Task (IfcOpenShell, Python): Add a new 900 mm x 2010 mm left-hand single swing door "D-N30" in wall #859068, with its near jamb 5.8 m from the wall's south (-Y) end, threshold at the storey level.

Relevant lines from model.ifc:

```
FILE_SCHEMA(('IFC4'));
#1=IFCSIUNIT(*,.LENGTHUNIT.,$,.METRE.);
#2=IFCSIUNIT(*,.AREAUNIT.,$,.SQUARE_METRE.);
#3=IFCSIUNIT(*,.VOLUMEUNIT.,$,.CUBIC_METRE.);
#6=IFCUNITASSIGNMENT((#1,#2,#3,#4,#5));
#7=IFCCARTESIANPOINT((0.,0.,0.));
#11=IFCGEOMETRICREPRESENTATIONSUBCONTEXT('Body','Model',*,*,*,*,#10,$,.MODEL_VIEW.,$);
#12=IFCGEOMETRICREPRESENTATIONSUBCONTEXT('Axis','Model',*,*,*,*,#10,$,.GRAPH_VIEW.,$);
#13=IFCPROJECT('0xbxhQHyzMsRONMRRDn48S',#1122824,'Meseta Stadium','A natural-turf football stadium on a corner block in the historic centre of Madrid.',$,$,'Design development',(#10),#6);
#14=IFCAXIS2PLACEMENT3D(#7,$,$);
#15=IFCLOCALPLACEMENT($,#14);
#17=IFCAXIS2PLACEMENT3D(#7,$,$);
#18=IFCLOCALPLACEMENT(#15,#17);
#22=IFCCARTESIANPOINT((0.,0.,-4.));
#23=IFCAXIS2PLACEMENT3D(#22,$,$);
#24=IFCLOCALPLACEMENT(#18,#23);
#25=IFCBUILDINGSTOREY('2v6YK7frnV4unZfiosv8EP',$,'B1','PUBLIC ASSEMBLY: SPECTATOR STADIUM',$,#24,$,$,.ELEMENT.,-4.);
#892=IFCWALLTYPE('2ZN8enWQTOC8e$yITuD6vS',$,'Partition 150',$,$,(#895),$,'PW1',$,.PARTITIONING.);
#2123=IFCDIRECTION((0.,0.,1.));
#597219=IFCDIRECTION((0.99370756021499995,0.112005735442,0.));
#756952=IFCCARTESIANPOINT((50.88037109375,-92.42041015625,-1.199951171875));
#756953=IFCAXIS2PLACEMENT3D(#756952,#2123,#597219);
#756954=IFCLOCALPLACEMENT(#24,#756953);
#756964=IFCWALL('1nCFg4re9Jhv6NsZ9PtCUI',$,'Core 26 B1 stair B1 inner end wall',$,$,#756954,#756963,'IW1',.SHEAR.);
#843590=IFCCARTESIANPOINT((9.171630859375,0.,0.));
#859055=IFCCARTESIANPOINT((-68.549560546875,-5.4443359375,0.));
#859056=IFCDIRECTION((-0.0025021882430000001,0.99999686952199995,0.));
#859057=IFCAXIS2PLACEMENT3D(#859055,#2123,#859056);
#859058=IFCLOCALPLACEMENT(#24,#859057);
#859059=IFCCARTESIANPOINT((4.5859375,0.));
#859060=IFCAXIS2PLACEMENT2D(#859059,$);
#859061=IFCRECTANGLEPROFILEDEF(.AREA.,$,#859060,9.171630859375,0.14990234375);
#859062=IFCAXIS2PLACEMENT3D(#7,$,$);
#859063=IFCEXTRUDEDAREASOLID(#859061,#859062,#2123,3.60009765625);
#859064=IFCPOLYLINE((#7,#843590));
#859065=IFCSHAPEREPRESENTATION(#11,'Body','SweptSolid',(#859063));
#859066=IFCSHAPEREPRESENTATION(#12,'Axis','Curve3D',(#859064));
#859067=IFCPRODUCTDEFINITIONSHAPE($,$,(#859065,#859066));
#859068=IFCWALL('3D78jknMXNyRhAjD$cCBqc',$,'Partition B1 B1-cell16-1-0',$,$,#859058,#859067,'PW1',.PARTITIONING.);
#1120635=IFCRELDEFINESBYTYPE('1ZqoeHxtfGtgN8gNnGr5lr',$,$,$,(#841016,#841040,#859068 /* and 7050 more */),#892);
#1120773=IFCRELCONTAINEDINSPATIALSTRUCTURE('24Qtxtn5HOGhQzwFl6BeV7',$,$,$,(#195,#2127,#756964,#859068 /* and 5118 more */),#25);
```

```python
import numpy as np
import ifcopenshell
import ifcopenshell.api.feature
import ifcopenshell.api.geometry
import ifcopenshell.api.root
import ifcopenshell.api.spatial
import ifcopenshell.geom
import ifcopenshell.util.element
import ifcopenshell.util.placement
import ifcopenshell.util.representation
import ifcopenshell.util.shape
import ifcopenshell.util.unit

model = ifcopenshell.open("model.ifc")
unit_scale = ifcopenshell.util.unit.calculate_unit_scale(model)
settings = ifcopenshell.geom.settings()


def volume(element):
    """Net volume in cubic metres, openings subtracted."""
    shape = ifcopenshell.geom.create_shape(settings, element)
    return ifcopenshell.util.shape.get_volume(shape.geometry)


wall = model.by_id(859068)
storey = ifcopenshell.util.element.get_container(wall, ifc_class="IfcBuildingStorey")
context = ifcopenshell.util.representation.get_context(model, "Model", "Body", "MODEL_VIEW")
before = volume(wall)

width, height, from_end, sill = 0.9, 2.01, 5.8, 0.0  # metres

# The wall runs along its own X axis, and the end named is its -X end.
wall_shape = ifcopenshell.geom.create_shape(settings, wall)
x, y, z = ifcopenshell.util.shape.get_vertices(wall_shape.geometry).T
start = x.min() + from_end
face, thickness = float(y.min()), float(y.max() - y.min())
wall_matrix = ifcopenshell.util.placement.get_local_placement(wall.ObjectPlacement)
level = ifcopenshell.util.placement.get_local_placement(storey.ObjectPlacement)[2, 3]


def in_wall(x, y):
    """Placement at x, y metres in the wall's axes, at sill height."""
    matrix = wall_matrix.copy()
    matrix[:, 3] = wall_matrix @ np.array([x / unit_scale, y / unit_scale, 0.0, 1.0])
    matrix[2, 3] = level + sill / unit_scale
    return matrix


# Opening: a box that overshoots both wall faces by 50 mm.
opening = ifcopenshell.api.root.create_entity(model, ifc_class="IfcOpeningElement", predefined_type="OPENING")
box = ifcopenshell.api.geometry.add_wall_representation(
    model, context=context, length=width, height=height, thickness=thickness + 0.1
)
ifcopenshell.api.geometry.assign_representation(model, product=opening, representation=box)
ifcopenshell.api.geometry.edit_object_placement(model, product=opening, matrix=in_wall(start, face - 0.05), is_si=False)
ifcopenshell.api.feature.add_feature(model, feature=opening, element=wall)

door = ifcopenshell.api.root.create_entity(model, ifc_class="IfcDoor", name="D-N30", predefined_type="DOOR")
door.OverallWidth, door.OverallHeight = width / unit_scale, height / unit_scale
door.OperationType = "SINGLE_SWING_LEFT"
body = ifcopenshell.api.geometry.add_door_representation(
    model,
    context=context,
    overall_width=door.OverallWidth,
    overall_height=door.OverallHeight,
    operation_type="SINGLE_SWING_LEFT",
    lining_properties={"LiningDepth": thickness / unit_scale, "ThresholdDepth": thickness / unit_scale},
)
ifcopenshell.api.geometry.assign_representation(model, product=door, representation=body)
ifcopenshell.api.spatial.assign_container(model, products=[door], relating_structure=storey)
ifcopenshell.api.feature.add_filling(model, opening=opening, element=door)

# The lining spans the wall, so the door starts at the wall face.
ifcopenshell.api.geometry.edit_object_placement(model, product=door, matrix=in_wall(start, face), is_si=False)

after = volume(wall)

print(f"wall volume {before:.3f} -> {after:.3f} m3")

model.write("model_rev.ifc")
```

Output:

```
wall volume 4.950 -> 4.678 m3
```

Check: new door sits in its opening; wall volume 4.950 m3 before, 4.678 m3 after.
